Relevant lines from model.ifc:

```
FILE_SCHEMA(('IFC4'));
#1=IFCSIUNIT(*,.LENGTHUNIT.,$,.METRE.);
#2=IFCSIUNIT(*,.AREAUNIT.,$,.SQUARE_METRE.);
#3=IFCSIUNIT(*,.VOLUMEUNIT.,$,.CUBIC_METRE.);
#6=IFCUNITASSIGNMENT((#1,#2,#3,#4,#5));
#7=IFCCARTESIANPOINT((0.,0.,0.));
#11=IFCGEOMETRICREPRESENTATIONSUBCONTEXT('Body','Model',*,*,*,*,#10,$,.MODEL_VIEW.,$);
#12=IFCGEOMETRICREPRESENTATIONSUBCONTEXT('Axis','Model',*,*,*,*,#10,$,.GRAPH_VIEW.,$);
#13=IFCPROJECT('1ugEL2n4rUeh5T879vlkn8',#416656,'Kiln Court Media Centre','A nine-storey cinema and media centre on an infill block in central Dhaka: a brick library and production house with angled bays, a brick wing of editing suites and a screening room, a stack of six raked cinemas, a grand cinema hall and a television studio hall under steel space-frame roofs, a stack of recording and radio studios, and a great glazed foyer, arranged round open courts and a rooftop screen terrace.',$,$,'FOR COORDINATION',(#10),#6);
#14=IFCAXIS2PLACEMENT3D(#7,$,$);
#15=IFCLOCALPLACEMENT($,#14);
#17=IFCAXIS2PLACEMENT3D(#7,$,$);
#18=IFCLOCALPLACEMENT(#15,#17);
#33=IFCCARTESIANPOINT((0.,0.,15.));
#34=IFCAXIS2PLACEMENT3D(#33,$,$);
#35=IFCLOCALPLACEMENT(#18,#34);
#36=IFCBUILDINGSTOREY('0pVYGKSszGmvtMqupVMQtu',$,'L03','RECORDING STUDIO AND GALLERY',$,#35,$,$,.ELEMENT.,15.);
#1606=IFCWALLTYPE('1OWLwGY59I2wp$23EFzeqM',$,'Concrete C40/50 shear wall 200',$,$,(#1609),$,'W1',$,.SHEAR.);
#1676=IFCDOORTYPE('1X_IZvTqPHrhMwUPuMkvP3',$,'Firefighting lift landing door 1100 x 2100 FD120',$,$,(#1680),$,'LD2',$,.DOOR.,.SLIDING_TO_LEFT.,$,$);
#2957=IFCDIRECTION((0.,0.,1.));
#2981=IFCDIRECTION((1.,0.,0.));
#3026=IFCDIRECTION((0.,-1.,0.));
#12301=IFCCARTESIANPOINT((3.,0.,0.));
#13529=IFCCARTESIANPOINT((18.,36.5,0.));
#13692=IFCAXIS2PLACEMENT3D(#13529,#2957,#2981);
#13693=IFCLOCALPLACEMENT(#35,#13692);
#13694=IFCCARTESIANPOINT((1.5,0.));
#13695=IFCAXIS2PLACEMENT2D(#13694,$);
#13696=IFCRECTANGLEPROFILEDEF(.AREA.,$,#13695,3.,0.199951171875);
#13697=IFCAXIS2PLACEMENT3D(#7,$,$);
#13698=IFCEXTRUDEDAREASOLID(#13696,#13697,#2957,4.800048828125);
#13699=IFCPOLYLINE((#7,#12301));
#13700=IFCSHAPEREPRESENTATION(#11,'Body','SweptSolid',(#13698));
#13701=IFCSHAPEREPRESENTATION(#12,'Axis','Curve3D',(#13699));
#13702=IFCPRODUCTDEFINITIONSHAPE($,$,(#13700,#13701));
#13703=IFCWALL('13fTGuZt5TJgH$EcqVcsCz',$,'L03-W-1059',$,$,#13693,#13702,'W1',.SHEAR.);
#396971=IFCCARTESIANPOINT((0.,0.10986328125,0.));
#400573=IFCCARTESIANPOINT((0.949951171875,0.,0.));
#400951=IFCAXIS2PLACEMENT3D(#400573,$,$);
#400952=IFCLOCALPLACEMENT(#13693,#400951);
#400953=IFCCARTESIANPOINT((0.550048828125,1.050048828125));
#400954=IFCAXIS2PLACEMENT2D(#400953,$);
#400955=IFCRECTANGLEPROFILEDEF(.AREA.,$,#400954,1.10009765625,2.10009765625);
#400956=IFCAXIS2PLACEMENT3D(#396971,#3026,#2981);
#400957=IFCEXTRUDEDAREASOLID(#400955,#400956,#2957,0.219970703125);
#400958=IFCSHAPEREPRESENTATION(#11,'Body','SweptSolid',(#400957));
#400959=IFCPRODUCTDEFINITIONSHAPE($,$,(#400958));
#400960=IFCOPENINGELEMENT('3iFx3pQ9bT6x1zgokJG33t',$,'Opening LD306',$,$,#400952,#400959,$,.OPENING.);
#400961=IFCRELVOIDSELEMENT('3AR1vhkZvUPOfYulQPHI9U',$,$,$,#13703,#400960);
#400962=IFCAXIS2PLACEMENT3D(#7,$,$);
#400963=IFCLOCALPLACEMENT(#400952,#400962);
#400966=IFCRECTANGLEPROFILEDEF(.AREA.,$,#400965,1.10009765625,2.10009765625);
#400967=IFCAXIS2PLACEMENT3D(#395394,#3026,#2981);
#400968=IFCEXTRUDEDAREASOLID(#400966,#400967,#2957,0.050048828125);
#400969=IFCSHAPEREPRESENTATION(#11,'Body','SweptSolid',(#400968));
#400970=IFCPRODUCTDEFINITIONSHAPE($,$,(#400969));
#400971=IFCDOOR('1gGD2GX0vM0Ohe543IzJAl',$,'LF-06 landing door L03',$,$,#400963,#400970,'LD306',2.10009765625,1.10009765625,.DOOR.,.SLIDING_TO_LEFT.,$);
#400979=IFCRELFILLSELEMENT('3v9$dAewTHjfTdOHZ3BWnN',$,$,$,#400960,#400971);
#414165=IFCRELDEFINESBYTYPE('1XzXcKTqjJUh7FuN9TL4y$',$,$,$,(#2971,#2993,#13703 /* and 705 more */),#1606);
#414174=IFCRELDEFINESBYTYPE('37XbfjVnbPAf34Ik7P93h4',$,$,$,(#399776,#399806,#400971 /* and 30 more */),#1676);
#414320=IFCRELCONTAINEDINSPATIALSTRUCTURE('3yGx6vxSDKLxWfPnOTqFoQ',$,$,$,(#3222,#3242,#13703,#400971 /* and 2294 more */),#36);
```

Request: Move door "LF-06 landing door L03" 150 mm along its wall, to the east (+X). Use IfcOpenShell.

```python
import ifcopenshell
import ifcopenshell.api.geometry
import ifcopenshell.util.placement

model = ifcopenshell.open("model.ifc")

door = model.by_guid("1gGD2GX0vM0Ohe543IzJAl")
opening = door.FillsVoids[0].RelatingOpeningElement
wall = opening.VoidsElements[0].RelatingBuildingElement

wall_matrix = ifcopenshell.util.placement.get_local_placement(wall.ObjectPlacement)
shift = wall_matrix[:3, 0] * 0.15
before = ifcopenshell.util.placement.get_local_placement(door.ObjectPlacement)[:3, 3].copy()

# The door is placed relative to its opening, so it follows when the opening moves.
matrix = ifcopenshell.util.placement.get_local_placement(opening.ObjectPlacement)
matrix[:3, 3] += shift
ifcopenshell.api.geometry.edit_object_placement(
    model, product=opening, matrix=matrix, is_si=False, should_transform_children=True
)

after = ifcopenshell.util.placement.get_local_placement(door.ObjectPlacement)[:3, 3]
print("door moved by", (after - before).round(3) + 0.0)

model.write("model_rev.ifc")
```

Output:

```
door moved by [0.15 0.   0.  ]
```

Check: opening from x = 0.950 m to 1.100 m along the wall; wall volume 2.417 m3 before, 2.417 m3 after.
